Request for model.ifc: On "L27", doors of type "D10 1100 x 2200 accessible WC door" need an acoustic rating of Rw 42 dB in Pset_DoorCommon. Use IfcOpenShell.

First a look at what the model holds.

```python
import ifcopenshell
import ifcopenshell.util.element

model = ifcopenshell.open("model.ifc")
print(model.schema)
storey = next(s for s in model.by_type("IfcBuildingStorey") if s.Name == "L27")
doors = [e for e in ifcopenshell.util.element.get_decomposition(storey) if e.is_a("IfcDoor")]
seen = {}
for e in doors:
    element_type = ifcopenshell.util.element.get_type(e)
    key = (element_type.Name if element_type != e and element_type else None, ifcopenshell.util.element.get_pset(e, "Pset_DoorCommon", "AcousticRating"))
    seen[key] = seen.get(key, 0) + 1
for (name, value), count in sorted(seen.items(), key=str):
    print(count, "x", name, "|", value)
```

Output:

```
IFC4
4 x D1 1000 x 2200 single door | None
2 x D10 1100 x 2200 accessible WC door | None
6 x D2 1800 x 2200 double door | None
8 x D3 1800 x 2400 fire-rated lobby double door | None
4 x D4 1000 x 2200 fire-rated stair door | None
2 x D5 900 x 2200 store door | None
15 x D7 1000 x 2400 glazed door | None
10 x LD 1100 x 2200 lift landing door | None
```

```python
import ifcopenshell
import ifcopenshell.api.pset
import ifcopenshell.util.element

model = ifcopenshell.open("model.ifc")

storey = next(s for s in model.by_type("IfcBuildingStorey") if s.Name == "L27")
doors = [e for e in ifcopenshell.util.element.get_decomposition(storey) if e.is_a("IfcDoor")]

count = 0
for e in doors:
    element_type = ifcopenshell.util.element.get_type(e)
    if element_type in (None, e) or element_type.Name != "D10 1100 x 2200 accessible WC door":
        continue
    # add_pset returns the element's existing set when there is one.
    pset = ifcopenshell.api.pset.add_pset(model, product=e, name="Pset_DoorCommon")
    ifcopenshell.api.pset.edit_pset(model, pset=pset, properties={"AcousticRating": "Rw 42 dB"})
    count += 1

print(count, "doors updated")

model.write("model_edited.ifc")
```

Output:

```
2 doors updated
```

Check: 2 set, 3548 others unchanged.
